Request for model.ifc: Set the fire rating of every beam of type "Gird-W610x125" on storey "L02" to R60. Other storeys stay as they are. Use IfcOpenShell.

First a look at what the model holds.

```python
import ifcopenshell
import ifcopenshell.util.element

model = ifcopenshell.open("model.ifc")
print(model.schema)
storey = next(s for s in model.by_type("IfcBuildingStorey") if s.Name == "L02")
beams = [e for e in ifcopenshell.util.element.get_decomposition(storey) if e.is_a("IfcBeam")]
seen = {}
for e in beams:
    element_type = ifcopenshell.util.element.get_type(e)
    key = (element_type.Name if element_type != e and element_type else None, ifcopenshell.util.element.get_pset(e, "Pset_BeamCommon", "FireRating"))
    seen[key] = seen.get(key, 0) + 1
for (name, value), count in sorted(seen.items(), key=str):
    print(count, "x", name, "|", value)
```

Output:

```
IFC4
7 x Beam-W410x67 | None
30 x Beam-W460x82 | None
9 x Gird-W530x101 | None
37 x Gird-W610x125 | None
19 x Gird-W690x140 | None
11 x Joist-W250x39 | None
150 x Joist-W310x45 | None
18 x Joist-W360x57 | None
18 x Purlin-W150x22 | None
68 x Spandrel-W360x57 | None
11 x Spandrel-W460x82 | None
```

```python
import ifcopenshell
import ifcopenshell.api.pset
import ifcopenshell.util.element

model = ifcopenshell.open("model.ifc")

storey = next(s for s in model.by_type("IfcBuildingStorey") if s.Name == "L02")
beams = [e for e in ifcopenshell.util.element.get_decomposition(storey) if e.is_a("IfcBeam")]

count = 0
for e in beams:
    element_type = ifcopenshell.util.element.get_type(e)
    if element_type in (None, e) or element_type.Name != "Gird-W610x125":
        continue
    # add_pset returns the element's existing set when there is one.
    pset = ifcopenshell.api.pset.add_pset(model, product=e, name="Pset_BeamCommon")
    ifcopenshell.api.pset.edit_pset(model, pset=pset, properties={"FireRating": "R60"})
    count += 1

print(count, "beams updated")

model.write("model_rev.ifc")
```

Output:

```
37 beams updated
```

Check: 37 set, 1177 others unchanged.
